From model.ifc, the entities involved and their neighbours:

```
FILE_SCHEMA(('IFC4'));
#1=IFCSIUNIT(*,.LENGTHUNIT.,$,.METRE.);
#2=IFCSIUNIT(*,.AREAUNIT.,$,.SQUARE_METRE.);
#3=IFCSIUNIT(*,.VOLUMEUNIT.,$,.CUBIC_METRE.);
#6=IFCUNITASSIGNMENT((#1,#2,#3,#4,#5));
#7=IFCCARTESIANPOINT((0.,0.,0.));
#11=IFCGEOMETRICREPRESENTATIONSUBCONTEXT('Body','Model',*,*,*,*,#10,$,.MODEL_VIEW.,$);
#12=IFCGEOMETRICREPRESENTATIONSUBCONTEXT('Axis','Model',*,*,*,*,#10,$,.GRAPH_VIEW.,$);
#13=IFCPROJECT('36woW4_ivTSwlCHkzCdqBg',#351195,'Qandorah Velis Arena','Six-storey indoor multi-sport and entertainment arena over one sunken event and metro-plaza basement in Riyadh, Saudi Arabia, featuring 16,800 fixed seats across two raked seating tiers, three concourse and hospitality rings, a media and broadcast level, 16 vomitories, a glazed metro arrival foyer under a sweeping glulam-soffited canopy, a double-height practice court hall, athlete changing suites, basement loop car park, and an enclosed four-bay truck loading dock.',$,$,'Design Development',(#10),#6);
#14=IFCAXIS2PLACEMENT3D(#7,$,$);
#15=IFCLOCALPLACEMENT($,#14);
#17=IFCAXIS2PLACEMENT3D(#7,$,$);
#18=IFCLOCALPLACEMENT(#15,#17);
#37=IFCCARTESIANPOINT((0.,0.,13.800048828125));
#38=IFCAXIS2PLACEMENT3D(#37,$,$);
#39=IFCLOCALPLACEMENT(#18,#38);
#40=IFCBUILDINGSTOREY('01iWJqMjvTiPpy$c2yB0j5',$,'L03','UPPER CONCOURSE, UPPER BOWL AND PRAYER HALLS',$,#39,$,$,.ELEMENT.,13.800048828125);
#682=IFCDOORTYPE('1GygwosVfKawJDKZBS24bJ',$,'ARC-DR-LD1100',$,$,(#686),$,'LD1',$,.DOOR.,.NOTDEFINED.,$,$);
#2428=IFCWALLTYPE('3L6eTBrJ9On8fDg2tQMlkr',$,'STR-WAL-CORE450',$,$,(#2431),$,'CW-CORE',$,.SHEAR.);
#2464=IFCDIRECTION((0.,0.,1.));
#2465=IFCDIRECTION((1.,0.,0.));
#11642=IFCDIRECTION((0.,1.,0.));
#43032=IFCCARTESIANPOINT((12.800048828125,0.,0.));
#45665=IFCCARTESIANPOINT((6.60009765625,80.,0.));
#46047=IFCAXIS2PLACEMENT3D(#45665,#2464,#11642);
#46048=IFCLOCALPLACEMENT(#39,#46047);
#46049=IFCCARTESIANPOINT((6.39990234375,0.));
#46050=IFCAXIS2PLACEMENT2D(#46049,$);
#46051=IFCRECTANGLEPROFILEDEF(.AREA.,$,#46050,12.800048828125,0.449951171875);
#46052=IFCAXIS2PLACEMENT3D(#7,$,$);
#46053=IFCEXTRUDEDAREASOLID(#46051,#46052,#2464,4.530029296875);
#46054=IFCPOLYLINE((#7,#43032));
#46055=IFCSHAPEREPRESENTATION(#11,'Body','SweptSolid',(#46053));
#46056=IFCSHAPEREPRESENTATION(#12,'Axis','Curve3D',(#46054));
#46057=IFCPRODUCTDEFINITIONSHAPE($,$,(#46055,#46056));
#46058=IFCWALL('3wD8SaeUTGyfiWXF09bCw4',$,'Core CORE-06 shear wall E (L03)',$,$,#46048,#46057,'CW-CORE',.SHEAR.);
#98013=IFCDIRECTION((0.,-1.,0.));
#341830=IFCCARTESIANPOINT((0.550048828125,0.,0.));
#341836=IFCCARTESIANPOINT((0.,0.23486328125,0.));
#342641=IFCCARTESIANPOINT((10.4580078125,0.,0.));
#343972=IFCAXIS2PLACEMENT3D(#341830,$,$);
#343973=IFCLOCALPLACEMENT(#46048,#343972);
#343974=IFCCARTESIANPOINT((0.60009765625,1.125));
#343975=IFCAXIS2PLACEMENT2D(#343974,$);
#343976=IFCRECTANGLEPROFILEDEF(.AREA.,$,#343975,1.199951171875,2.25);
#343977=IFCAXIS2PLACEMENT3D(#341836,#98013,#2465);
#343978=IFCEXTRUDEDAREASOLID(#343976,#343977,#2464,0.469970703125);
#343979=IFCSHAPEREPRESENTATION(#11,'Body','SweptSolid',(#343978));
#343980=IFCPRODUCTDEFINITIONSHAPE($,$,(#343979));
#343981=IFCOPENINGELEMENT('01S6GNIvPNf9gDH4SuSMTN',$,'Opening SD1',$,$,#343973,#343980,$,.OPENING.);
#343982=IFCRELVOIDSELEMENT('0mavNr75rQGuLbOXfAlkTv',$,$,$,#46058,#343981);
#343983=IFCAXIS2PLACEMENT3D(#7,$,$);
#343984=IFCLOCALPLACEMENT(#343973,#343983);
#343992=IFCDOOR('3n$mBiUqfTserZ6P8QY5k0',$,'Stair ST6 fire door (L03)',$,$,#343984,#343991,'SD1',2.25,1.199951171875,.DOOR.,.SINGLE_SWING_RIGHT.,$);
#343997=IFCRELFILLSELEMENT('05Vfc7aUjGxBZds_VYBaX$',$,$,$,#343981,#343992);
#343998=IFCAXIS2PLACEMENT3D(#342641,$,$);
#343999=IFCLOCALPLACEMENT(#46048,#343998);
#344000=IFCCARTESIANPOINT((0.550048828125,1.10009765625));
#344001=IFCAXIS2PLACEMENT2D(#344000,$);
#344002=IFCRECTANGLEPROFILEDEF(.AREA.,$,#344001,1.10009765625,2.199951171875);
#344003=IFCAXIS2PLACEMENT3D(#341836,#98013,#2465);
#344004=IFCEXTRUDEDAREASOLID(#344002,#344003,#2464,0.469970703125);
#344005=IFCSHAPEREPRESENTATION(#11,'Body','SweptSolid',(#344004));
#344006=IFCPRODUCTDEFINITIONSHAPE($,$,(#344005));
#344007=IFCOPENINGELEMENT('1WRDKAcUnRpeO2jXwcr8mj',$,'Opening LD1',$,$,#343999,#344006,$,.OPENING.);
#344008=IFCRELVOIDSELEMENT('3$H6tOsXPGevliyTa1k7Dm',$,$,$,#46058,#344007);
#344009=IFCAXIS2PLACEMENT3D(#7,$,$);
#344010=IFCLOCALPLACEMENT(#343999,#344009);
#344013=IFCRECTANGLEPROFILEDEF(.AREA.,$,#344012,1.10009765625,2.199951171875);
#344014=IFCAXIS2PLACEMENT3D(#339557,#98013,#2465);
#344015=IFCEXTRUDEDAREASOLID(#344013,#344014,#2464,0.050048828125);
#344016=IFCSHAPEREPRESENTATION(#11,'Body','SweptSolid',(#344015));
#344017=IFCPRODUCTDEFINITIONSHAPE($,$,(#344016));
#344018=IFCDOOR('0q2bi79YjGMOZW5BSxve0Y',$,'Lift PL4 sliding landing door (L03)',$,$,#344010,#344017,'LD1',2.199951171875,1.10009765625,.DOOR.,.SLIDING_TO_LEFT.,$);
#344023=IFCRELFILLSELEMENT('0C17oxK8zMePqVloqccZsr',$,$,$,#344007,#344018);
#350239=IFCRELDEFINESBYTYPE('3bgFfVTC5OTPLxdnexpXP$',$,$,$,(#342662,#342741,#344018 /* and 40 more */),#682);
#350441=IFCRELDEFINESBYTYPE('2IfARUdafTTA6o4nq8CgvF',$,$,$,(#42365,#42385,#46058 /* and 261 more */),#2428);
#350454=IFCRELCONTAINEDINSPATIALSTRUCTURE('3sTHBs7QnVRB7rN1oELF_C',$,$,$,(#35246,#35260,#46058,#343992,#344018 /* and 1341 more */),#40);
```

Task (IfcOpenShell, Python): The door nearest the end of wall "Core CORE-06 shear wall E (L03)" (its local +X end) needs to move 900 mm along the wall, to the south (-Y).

```python
import ifcopenshell
import ifcopenshell.api.geometry
import ifcopenshell.util.placement
import ifcopenshell.util.unit

model = ifcopenshell.open("model.ifc")
unit_scale = ifcopenshell.util.unit.calculate_unit_scale(model)

door = model.by_guid("0q2bi79YjGMOZW5BSxve0Y")
opening = door.FillsVoids[0].RelatingOpeningElement
wall = opening.VoidsElements[0].RelatingBuildingElement

wall_matrix = ifcopenshell.util.placement.get_local_placement(wall.ObjectPlacement)
shift = wall_matrix[:3, 0] * -0.9 / unit_scale
before = ifcopenshell.util.placement.get_local_placement(door.ObjectPlacement)[:3, 3].copy()

# The door is placed relative to its opening, so it follows when the opening moves.
matrix = ifcopenshell.util.placement.get_local_placement(opening.ObjectPlacement)
matrix[:3, 3] += shift
ifcopenshell.api.geometry.edit_object_placement(
    model, product=opening, matrix=matrix, is_si=False, should_transform_children=True
)

after = ifcopenshell.util.placement.get_local_placement(door.ObjectPlacement)[:3, 3]
print("door moved by", (after - before).round(3) + 0.0)

model.write("model_rev.ifc")
```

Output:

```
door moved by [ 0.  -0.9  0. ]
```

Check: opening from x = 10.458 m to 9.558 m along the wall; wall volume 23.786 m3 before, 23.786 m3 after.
